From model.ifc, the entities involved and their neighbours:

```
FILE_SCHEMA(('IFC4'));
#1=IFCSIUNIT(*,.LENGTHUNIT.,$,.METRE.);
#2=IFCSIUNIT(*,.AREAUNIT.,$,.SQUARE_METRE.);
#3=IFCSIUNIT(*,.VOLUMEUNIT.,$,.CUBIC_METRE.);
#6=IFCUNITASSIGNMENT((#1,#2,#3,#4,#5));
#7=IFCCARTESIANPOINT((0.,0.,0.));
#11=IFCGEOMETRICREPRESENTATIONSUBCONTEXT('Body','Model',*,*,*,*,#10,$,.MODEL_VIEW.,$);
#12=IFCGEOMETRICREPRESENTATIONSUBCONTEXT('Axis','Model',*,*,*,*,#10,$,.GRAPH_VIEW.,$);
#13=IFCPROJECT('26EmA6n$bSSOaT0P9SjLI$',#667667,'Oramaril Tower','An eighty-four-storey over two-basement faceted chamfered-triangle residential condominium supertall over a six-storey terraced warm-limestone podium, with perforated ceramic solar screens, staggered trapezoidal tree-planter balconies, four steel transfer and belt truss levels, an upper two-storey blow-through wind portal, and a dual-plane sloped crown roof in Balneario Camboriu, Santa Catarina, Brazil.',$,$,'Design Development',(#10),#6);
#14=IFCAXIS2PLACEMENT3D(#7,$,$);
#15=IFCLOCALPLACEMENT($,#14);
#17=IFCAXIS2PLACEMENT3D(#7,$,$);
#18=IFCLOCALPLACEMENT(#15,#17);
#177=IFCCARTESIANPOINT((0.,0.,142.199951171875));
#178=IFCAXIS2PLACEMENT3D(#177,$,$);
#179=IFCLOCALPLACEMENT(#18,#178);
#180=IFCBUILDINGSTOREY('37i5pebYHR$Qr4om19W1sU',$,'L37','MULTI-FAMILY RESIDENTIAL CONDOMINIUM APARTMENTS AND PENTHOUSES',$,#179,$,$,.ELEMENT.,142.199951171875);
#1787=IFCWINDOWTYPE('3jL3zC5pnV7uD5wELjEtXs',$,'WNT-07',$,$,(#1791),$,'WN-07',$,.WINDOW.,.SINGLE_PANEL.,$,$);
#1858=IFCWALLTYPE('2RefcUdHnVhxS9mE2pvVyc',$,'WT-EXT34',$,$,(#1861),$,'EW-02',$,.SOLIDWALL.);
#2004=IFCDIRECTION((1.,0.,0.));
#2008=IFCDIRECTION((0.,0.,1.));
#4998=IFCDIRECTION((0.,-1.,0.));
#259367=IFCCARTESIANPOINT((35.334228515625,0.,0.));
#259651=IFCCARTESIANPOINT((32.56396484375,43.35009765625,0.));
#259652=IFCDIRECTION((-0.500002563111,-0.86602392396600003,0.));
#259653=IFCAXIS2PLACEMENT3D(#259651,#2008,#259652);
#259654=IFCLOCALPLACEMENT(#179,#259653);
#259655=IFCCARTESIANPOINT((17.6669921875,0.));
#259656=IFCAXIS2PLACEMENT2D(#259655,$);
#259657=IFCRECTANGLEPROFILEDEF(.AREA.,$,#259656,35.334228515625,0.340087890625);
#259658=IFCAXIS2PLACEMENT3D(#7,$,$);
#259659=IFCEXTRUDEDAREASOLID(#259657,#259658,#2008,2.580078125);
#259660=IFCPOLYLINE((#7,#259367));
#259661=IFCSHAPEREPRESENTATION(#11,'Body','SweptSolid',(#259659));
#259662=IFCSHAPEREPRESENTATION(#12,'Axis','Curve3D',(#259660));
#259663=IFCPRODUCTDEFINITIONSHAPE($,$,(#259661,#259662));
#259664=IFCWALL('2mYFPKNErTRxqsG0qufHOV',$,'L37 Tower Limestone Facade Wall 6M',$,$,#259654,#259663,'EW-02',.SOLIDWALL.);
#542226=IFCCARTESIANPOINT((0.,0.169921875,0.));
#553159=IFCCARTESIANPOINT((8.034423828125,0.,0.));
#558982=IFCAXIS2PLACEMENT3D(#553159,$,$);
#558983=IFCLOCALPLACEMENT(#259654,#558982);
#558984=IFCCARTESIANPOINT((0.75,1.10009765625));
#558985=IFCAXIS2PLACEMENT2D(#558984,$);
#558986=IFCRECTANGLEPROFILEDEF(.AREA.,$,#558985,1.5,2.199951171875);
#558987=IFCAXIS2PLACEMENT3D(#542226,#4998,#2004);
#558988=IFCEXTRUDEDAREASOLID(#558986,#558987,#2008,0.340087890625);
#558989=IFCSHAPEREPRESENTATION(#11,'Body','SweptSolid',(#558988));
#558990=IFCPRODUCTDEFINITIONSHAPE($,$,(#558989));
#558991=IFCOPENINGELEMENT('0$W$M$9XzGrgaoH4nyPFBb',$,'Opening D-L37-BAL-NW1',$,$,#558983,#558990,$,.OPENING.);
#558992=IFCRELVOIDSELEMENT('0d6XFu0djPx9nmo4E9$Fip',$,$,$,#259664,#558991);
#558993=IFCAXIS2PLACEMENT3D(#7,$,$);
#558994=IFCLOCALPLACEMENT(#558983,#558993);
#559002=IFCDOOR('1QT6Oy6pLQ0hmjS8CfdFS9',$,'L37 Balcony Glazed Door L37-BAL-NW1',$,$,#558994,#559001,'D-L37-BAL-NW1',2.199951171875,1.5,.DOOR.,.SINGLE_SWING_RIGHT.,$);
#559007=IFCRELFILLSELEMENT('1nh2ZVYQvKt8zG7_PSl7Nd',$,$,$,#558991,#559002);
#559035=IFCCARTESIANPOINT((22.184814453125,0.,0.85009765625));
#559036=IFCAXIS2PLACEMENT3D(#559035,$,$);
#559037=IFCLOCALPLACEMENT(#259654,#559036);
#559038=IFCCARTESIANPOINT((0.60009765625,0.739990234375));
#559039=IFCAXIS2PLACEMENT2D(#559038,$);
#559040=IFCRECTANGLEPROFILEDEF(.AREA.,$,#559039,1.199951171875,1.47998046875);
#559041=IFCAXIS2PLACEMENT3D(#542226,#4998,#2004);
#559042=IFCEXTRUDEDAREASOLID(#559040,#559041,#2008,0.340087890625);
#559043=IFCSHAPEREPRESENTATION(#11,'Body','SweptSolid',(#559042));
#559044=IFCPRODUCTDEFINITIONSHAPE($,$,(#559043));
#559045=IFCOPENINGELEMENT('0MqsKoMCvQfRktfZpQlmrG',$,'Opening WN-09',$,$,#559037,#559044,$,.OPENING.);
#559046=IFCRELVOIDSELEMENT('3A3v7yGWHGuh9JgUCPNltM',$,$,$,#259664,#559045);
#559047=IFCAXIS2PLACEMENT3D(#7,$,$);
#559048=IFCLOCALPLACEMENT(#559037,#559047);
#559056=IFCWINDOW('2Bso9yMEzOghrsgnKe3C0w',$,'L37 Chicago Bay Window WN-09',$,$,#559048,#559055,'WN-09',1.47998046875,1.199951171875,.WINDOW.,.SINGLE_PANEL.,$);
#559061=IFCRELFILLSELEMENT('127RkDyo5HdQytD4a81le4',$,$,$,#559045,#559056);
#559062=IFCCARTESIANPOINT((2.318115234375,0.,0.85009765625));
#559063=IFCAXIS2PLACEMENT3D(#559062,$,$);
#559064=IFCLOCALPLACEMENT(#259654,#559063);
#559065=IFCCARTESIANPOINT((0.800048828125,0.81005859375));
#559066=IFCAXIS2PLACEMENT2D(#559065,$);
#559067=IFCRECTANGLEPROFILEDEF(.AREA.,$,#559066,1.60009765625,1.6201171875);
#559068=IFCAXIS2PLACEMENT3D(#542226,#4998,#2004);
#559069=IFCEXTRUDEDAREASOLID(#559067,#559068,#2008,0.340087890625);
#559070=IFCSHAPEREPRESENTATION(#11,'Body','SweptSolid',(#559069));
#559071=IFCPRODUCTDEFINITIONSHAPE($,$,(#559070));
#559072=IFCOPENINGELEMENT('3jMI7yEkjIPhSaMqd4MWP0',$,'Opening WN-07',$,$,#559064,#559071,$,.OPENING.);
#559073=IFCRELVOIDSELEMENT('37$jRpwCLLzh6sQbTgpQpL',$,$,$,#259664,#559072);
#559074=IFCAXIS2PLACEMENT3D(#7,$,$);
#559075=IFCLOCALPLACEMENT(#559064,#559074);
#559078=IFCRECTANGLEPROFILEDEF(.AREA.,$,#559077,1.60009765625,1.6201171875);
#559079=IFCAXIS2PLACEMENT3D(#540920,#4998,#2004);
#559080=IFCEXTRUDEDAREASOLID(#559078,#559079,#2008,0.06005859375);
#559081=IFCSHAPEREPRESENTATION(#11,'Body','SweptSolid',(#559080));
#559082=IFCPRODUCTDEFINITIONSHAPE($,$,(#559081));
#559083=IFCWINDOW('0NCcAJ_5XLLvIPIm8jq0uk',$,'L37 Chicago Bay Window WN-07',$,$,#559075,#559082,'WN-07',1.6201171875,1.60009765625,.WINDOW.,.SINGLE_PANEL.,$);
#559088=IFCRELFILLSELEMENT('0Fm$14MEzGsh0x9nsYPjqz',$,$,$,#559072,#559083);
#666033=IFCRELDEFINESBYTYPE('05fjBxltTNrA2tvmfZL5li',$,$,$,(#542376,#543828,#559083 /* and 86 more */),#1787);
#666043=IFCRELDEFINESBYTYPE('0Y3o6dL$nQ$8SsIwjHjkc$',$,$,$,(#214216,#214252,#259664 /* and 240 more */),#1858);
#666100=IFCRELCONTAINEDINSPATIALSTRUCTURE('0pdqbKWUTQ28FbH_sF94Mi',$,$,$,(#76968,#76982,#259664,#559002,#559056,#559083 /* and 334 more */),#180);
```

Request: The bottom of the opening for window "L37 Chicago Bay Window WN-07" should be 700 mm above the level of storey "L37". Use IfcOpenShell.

```python
import numpy as np
import ifcopenshell
import ifcopenshell.api.geometry
import ifcopenshell.geom
import ifcopenshell.util.element
import ifcopenshell.util.placement
import ifcopenshell.util.shape
import ifcopenshell.util.unit

model = ifcopenshell.open("model.ifc")
unit_scale = ifcopenshell.util.unit.calculate_unit_scale(model)

window = model.by_guid("0NCcAJ_5XLLvIPIm8jq0uk")
opening = window.FillsVoids[0].RelatingOpeningElement
storey = ifcopenshell.util.element.get_container(window, ifc_class="IfcBuildingStorey")
level = ifcopenshell.util.placement.get_local_placement(storey.ObjectPlacement)[2, 3]

# The opening's origin need not be at the sill, so measure its lowest point.
shape = ifcopenshell.geom.create_shape(ifcopenshell.geom.settings(), opening)
bottom = ifcopenshell.util.shape.get_shape_bottom_elevation(shape, shape.geometry) / unit_scale
dz = level + 0.7 / unit_scale - bottom

shift = np.array([0.0, 0.0, dz])
# The window is placed relative to its opening, so it follows when the opening moves.
matrix = ifcopenshell.util.placement.get_local_placement(opening.ObjectPlacement)
matrix[:3, 3] += shift
ifcopenshell.api.geometry.edit_object_placement(
    model, product=opening, matrix=matrix, is_si=False, should_transform_children=True
)

print(f"moved by {dz * unit_scale:+.3f} m")

model.write("model-out.ifc")
```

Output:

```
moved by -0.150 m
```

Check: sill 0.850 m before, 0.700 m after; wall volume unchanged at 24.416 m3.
